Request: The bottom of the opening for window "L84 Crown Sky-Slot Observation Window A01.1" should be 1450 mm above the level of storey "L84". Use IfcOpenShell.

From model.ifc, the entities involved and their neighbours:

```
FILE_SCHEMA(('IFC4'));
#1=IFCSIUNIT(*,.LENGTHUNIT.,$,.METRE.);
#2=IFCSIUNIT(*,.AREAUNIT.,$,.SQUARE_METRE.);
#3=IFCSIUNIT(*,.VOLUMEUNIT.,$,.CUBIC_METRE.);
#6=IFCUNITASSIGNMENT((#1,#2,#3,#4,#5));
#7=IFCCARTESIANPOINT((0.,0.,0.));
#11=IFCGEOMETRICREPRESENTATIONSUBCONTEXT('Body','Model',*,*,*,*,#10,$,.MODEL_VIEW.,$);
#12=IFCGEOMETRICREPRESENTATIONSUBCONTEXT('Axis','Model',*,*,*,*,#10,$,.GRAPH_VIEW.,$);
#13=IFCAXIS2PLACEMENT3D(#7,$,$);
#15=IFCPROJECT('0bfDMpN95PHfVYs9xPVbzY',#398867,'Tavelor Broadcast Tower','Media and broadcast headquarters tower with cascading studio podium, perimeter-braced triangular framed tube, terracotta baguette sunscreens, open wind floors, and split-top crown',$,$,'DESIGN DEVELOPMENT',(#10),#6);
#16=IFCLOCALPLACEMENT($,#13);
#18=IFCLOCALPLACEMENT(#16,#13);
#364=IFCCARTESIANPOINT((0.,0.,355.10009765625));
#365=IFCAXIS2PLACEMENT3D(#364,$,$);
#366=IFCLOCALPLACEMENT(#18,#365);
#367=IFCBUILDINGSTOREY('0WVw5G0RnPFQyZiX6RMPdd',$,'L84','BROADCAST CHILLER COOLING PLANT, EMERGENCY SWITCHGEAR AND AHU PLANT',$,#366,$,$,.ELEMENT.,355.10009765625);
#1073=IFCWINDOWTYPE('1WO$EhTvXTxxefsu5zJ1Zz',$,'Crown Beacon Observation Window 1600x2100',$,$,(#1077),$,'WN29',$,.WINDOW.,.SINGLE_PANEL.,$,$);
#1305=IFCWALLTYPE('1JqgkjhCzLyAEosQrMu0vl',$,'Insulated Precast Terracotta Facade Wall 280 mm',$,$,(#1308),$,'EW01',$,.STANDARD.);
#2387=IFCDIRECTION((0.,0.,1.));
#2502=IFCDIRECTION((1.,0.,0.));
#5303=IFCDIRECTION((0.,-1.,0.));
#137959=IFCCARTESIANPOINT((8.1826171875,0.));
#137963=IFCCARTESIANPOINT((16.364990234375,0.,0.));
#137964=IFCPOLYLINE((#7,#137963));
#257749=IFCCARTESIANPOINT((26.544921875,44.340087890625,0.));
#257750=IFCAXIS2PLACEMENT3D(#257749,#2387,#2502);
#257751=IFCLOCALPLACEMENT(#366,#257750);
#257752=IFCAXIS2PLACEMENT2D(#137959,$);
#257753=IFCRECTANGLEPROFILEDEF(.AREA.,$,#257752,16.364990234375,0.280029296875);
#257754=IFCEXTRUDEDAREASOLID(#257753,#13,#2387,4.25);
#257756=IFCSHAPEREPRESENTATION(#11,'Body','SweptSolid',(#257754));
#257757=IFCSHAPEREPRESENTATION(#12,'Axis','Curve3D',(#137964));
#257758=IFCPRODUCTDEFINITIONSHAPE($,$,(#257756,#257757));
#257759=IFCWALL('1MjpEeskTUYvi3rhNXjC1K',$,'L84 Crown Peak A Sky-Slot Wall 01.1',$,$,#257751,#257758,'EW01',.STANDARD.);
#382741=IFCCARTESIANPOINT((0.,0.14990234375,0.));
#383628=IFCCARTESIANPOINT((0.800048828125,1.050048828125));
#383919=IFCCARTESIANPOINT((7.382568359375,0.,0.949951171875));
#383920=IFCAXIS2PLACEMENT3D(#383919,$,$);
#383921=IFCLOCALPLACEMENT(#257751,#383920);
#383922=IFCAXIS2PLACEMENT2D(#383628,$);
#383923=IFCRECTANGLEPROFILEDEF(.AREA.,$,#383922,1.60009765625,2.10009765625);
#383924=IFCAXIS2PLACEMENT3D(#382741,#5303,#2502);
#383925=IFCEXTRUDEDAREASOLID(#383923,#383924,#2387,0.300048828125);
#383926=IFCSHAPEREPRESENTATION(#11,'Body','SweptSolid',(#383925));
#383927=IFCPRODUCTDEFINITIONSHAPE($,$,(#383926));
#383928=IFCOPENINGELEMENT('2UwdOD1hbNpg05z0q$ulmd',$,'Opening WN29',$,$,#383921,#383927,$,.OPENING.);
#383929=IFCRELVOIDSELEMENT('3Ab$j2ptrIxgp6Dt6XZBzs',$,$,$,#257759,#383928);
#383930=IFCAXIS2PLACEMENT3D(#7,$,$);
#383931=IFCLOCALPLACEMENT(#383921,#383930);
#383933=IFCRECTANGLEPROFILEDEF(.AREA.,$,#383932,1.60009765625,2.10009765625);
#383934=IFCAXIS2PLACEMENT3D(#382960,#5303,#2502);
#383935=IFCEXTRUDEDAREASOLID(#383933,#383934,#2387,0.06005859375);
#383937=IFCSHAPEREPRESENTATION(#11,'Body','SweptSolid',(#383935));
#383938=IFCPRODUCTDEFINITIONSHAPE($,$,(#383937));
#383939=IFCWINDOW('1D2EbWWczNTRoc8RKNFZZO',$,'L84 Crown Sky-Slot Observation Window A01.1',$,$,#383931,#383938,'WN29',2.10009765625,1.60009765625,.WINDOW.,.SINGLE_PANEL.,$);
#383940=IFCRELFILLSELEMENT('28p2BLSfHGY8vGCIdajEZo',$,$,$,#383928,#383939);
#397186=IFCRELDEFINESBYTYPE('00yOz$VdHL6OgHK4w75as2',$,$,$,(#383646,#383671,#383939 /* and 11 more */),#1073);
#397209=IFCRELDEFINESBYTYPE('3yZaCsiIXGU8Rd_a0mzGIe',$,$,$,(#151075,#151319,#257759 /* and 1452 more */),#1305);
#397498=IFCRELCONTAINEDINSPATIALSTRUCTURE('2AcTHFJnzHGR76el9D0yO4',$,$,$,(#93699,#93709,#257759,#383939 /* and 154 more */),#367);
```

```python
import numpy as np
import ifcopenshell
import ifcopenshell.api.geometry
import ifcopenshell.geom
import ifcopenshell.util.element
import ifcopenshell.util.placement
import ifcopenshell.util.shape
import ifcopenshell.util.unit

model = ifcopenshell.open("model.ifc")
unit_scale = ifcopenshell.util.unit.calculate_unit_scale(model)

window = model.by_guid("1D2EbWWczNTRoc8RKNFZZO")
opening = window.FillsVoids[0].RelatingOpeningElement
storey = ifcopenshell.util.element.get_container(window, ifc_class="IfcBuildingStorey")
level = ifcopenshell.util.placement.get_local_placement(storey.ObjectPlacement)[2, 3]

# The opening's origin need not be at the sill, so measure its lowest point.
shape = ifcopenshell.geom.create_shape(ifcopenshell.geom.settings(), opening)
bottom = ifcopenshell.util.shape.get_shape_bottom_elevation(shape, shape.geometry) / unit_scale
dz = level + 1.45 / unit_scale - bottom

shift = np.array([0.0, 0.0, dz])
# The window is placed relative to its opening, so it follows when the opening moves.
matrix = ifcopenshell.util.placement.get_local_placement(opening.ObjectPlacement)
matrix[:3, 3] += shift
ifcopenshell.api.geometry.edit_object_placement(
    model, product=opening, matrix=matrix, is_si=False, should_transform_children=True
)

print(f"moved by {dz * unit_scale:+.3f} m")

model.write("model_updated.ifc")
```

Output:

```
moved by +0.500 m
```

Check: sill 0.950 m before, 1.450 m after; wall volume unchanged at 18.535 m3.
